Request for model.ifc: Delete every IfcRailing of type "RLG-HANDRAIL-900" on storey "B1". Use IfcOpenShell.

First a look at what the model holds.

```python
import ifcopenshell
import ifcopenshell.util.element

model = ifcopenshell.open("model.ifc")
print(model.schema)
storey = next(s for s in model.by_type("IfcBuildingStorey") if s.Name == "B1")
railings = [e for e in ifcopenshell.util.element.get_decomposition(storey) if e.is_a("IfcRailing")]
seen = {}
for e in railings:
    element_type = ifcopenshell.util.element.get_type(e)
    name = element_type.Name if element_type not in (None, e) else None
    seen[name] = seen.get(name, 0) + 1
for name, count in sorted(seen.items(), key=str):
    print(count, "x", name)
```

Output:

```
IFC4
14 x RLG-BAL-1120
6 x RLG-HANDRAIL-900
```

```python
import ifcopenshell
import ifcopenshell.api.root
import ifcopenshell.util.element

model = ifcopenshell.open("model.ifc")

storey = next(s for s in model.by_type("IfcBuildingStorey") if s.Name == "B1")
railings = [e for e in ifcopenshell.util.element.get_decomposition(storey) if e.is_a("IfcRailing")]
targets = [e for e in railings if (t := ifcopenshell.util.element.get_type(e)) not in (None, e) and t.Name == "RLG-HANDRAIL-900"]

for e in targets:
    ifcopenshell.api.root.remove_product(model, product=e)
print(len(targets), "removed")

model.write("model_v2.ifc")
```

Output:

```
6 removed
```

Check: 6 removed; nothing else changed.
